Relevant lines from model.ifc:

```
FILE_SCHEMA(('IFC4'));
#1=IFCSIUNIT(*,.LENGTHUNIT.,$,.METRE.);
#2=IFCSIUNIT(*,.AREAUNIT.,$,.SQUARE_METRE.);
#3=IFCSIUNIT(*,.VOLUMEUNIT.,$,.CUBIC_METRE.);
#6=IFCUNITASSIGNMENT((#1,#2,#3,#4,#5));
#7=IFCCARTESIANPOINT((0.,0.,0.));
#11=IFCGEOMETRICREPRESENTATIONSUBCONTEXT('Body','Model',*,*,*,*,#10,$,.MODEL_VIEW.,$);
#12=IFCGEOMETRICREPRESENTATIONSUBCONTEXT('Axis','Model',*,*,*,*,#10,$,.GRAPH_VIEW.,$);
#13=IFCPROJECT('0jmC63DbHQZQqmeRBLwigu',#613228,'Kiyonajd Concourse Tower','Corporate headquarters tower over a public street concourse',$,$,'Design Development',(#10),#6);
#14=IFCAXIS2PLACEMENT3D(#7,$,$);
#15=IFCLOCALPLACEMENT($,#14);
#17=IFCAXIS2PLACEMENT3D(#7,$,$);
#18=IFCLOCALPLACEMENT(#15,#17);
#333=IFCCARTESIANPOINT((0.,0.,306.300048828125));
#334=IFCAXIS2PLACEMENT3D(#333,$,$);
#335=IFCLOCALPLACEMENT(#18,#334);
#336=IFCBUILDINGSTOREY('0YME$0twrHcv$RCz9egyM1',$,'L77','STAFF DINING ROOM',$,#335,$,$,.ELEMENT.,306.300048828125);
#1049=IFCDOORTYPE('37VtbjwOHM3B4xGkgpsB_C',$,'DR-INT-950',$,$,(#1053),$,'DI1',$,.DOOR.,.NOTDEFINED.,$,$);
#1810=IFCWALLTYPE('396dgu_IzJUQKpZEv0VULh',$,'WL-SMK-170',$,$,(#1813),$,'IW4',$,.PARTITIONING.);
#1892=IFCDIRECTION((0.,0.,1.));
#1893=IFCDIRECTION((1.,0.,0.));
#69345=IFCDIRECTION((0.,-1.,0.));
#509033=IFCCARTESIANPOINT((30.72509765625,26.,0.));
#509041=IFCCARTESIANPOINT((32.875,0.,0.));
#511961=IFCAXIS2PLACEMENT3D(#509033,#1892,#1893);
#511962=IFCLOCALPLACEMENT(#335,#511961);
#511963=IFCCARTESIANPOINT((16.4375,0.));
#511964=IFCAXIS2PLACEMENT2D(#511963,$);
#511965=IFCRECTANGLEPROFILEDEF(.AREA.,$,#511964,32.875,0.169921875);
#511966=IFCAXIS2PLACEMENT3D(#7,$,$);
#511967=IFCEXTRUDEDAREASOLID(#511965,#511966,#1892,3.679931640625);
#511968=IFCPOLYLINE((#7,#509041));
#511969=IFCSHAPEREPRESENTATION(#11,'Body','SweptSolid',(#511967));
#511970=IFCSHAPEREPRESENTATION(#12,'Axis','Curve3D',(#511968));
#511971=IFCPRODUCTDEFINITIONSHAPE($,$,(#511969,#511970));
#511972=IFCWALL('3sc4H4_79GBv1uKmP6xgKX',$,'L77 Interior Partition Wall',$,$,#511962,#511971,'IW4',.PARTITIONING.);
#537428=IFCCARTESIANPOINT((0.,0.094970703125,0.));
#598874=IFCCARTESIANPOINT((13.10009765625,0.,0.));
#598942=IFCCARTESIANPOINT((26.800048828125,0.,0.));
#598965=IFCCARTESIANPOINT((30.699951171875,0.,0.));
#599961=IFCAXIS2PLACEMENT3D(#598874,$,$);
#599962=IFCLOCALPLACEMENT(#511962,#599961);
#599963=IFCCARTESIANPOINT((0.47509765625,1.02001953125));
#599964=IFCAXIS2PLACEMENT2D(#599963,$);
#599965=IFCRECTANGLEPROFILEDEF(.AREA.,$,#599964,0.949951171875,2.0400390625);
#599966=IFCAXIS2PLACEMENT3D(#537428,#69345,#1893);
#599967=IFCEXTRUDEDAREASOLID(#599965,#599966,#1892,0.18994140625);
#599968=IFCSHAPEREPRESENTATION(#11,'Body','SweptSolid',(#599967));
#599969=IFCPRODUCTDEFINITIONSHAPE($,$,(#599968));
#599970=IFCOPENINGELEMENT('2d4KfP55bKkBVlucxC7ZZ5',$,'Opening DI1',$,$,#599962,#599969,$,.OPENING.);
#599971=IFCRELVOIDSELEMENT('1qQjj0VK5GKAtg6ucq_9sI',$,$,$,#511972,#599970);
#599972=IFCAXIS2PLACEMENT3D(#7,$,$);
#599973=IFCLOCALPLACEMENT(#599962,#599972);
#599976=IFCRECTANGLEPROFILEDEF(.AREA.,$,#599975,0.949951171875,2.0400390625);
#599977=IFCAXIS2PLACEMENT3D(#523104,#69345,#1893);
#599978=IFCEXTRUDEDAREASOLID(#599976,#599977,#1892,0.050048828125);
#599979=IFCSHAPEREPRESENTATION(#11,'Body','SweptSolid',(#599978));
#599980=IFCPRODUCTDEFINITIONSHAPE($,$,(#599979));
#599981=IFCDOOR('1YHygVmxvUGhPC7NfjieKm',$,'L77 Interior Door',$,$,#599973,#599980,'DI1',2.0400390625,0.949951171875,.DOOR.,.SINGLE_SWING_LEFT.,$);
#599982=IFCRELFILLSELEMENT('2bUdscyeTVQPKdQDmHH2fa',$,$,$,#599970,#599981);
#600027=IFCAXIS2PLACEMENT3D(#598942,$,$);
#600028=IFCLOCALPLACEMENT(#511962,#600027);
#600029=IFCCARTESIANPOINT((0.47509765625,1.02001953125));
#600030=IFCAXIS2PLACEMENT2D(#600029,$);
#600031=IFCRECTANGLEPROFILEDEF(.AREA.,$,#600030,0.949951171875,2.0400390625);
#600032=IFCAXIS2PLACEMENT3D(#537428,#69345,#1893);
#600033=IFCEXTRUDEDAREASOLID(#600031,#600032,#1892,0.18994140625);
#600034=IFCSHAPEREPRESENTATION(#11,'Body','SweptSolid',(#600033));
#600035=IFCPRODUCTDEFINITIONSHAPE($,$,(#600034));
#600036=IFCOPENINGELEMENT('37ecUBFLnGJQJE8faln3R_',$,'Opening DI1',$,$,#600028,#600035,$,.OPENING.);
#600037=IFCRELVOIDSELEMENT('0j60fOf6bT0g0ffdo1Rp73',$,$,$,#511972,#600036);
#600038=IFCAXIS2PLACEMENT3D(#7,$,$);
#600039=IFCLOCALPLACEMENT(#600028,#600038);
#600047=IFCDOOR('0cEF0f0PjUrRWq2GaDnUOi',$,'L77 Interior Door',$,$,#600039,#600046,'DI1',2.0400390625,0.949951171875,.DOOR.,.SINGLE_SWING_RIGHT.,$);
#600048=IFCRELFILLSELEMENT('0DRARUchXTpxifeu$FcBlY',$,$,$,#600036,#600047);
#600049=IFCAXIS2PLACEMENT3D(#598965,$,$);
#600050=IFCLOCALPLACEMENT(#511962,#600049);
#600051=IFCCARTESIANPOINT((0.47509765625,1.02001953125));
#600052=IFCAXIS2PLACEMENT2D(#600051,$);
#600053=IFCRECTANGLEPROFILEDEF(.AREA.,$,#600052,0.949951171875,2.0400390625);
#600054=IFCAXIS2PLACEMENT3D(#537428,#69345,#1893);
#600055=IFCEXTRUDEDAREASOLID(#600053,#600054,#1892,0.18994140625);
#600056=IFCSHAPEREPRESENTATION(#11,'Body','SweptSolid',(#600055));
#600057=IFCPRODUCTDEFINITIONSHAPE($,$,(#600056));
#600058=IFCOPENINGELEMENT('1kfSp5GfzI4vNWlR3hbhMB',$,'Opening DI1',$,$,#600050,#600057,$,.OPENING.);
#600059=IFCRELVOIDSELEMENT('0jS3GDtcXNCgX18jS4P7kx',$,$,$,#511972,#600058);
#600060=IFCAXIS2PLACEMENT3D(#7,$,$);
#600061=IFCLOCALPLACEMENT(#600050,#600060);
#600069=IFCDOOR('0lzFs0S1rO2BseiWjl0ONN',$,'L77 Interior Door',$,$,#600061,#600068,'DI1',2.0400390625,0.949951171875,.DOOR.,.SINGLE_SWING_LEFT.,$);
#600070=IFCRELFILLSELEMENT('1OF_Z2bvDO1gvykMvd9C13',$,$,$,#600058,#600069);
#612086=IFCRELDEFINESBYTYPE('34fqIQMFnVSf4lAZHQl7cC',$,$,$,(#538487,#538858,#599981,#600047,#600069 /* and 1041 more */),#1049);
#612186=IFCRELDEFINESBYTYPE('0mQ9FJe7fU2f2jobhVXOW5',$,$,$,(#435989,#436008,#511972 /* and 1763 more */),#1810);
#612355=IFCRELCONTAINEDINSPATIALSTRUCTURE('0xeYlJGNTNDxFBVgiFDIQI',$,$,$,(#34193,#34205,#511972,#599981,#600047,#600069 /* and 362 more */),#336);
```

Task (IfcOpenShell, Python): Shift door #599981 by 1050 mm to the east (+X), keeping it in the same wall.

```python
import ifcopenshell
import ifcopenshell.api.geometry
import ifcopenshell.util.placement
import ifcopenshell.util.unit

model = ifcopenshell.open("model.ifc")
unit_scale = ifcopenshell.util.unit.calculate_unit_scale(model)

door = model.by_id(599981)
opening = door.FillsVoids[0].RelatingOpeningElement
wall = opening.VoidsElements[0].RelatingBuildingElement

wall_matrix = ifcopenshell.util.placement.get_local_placement(wall.ObjectPlacement)
shift = wall_matrix[:3, 0] * 1.05 / unit_scale
before = ifcopenshell.util.placement.get_local_placement(door.ObjectPlacement)[:3, 3].copy()

# The door is placed relative to its opening, so it follows when the opening moves.
matrix = ifcopenshell.util.placement.get_local_placement(opening.ObjectPlacement)
matrix[:3, 3] += shift
ifcopenshell.api.geometry.edit_object_placement(
    model, product=opening, matrix=matrix, is_si=False, should_transform_children=True
)

after = ifcopenshell.util.placement.get_local_placement(door.ObjectPlacement)[:3, 3]
print("door moved by", (after - before).round(3) + 0.0)

model.write("model_rev.ifc")
```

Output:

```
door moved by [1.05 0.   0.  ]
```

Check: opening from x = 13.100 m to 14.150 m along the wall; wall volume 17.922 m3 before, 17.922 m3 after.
